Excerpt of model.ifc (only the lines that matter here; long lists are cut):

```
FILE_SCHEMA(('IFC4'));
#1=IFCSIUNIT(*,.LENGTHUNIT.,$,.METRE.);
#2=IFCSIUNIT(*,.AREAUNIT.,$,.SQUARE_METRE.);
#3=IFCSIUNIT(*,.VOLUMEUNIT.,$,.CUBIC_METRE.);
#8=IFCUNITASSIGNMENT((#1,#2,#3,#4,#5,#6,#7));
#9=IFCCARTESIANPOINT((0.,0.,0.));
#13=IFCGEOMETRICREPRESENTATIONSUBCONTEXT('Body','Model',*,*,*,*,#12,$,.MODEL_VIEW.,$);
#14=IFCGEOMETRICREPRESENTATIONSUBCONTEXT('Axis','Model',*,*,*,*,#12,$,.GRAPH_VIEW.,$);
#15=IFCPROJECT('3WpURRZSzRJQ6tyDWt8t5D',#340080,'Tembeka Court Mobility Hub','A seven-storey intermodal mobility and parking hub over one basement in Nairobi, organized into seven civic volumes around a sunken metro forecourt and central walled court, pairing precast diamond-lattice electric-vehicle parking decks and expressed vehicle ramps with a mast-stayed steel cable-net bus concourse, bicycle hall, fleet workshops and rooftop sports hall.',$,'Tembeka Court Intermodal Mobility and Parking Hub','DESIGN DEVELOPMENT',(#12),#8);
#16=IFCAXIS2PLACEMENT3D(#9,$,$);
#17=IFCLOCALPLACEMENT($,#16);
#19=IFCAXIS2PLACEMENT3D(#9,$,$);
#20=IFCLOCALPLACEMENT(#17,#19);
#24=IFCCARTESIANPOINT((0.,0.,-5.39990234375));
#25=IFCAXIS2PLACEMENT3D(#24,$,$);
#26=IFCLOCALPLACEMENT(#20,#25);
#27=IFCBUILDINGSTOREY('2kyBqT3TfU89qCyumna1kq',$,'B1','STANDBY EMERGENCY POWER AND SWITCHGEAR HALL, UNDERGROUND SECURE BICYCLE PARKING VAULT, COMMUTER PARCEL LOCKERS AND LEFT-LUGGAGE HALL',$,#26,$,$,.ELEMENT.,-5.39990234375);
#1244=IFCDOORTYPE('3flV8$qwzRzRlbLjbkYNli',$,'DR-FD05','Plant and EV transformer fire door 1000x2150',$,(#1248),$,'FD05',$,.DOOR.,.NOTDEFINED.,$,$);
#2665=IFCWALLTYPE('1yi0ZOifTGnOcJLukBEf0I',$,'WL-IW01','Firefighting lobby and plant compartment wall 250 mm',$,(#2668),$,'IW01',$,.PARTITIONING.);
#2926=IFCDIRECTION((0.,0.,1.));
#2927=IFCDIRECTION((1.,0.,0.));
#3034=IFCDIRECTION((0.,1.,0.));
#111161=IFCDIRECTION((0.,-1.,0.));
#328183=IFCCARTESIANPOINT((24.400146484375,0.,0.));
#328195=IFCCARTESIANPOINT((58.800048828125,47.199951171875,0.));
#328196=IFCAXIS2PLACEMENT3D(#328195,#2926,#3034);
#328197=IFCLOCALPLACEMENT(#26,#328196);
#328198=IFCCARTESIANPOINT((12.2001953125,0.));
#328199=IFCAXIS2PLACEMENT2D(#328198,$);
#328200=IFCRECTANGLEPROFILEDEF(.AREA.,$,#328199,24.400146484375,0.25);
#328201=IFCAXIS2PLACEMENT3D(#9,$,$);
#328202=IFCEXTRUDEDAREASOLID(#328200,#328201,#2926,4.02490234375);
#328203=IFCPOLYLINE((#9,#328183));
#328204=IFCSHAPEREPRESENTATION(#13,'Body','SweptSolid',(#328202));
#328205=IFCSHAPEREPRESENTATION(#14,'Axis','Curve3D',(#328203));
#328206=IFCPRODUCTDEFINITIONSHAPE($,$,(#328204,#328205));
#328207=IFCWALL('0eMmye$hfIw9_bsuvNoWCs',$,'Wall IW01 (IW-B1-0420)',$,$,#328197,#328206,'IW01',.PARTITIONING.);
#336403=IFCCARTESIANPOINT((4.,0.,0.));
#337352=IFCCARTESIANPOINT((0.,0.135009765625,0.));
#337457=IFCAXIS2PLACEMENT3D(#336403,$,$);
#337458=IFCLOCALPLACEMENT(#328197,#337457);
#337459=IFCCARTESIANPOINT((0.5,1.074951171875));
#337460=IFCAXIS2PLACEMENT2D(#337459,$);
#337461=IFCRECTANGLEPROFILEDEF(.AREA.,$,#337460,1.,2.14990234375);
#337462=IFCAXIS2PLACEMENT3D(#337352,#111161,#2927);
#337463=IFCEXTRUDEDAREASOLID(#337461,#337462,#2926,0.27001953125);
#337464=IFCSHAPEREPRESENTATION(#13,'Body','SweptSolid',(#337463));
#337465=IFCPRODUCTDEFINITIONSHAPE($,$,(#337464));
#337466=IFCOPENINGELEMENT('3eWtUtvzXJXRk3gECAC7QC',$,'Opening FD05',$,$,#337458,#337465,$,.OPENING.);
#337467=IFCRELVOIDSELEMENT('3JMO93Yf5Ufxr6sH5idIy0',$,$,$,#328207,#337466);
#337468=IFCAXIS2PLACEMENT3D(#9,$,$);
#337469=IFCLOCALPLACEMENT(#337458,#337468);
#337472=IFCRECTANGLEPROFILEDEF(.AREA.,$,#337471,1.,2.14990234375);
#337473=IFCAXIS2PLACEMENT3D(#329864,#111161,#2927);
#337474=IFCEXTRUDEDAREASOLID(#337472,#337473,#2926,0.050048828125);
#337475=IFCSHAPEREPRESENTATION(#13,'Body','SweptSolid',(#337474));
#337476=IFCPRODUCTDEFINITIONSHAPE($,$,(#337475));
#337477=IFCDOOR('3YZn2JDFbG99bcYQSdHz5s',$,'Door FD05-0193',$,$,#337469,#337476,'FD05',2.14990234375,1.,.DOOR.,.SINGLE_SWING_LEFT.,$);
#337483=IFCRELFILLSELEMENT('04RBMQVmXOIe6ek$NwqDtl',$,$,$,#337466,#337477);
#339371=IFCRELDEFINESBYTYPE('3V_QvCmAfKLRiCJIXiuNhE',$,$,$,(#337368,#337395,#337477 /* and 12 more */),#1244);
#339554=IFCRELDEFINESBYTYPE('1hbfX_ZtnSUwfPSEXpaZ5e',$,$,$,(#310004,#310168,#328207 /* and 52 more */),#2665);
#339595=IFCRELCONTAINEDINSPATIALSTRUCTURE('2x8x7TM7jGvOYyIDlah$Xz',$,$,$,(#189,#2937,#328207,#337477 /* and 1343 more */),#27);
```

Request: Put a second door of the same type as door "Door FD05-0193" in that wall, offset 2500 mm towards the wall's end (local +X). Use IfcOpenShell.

```python
import ifcopenshell
import ifcopenshell.api.feature
import ifcopenshell.api.geometry
import ifcopenshell.api.root
import ifcopenshell.geom
import ifcopenshell.util.element
import ifcopenshell.util.placement
import ifcopenshell.util.shape

model = ifcopenshell.open("model.ifc")
settings = ifcopenshell.geom.settings()


def volume(element):
    """Net volume in cubic metres, openings subtracted."""
    shape = ifcopenshell.geom.create_shape(settings, element)
    return ifcopenshell.util.shape.get_volume(shape.geometry)


door = model.by_id(337477)
opening = door.FillsVoids[0].RelatingOpeningElement
wall = opening.VoidsElements[0].RelatingBuildingElement
before = volume(wall)
shift = ifcopenshell.util.placement.get_local_placement(wall.ObjectPlacement)[:3, 0] * 2.5

# copy_class copies the void relationship, type, container and properties, but no geometry.
new_opening = ifcopenshell.api.root.copy_class(model, product=opening)
new_opening.Representation = ifcopenshell.util.element.copy_deep(
    model, opening.Representation, exclude=["IfcGeometricRepresentationContext", "IfcRepresentationMap"]
)
new_door = ifcopenshell.api.root.copy_class(model, product=door)
new_door.Representation = ifcopenshell.util.element.copy_deep(
    model, door.Representation, exclude=["IfcGeometricRepresentationContext", "IfcRepresentationMap"]
)
new_door.Tag = None
ifcopenshell.api.feature.add_filling(model, opening=new_opening, element=new_door)

for old, new in ((opening, new_opening), (door, new_door)):
    matrix = ifcopenshell.util.placement.get_local_placement(old.ObjectPlacement)
    matrix[:3, 3] += shift
    ifcopenshell.api.geometry.edit_object_placement(model, product=new, matrix=matrix, is_si=False)

after = volume(wall)

print(f"wall volume {before:.3f} -> {after:.3f} m3")

model.write("model-out.ifc")
```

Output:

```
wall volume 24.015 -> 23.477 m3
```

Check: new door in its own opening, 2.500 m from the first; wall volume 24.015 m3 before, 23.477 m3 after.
